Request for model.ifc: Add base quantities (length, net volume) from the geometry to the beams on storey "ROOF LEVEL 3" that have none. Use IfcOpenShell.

First a look at what the model holds.

```python
import ifcopenshell
import ifcopenshell.util.element
import ifcopenshell.util.unit

model = ifcopenshell.open("model.ifc")
print(model.schema)
for unit_type in ("LENGTHUNIT", "AREAUNIT", "VOLUMEUNIT"):
    print(unit_type, ifcopenshell.util.unit.calculate_unit_scale(model, unit_type))
storey = next(s for s in model.by_type("IfcBuildingStorey") if s.Name == "ROOF LEVEL 3")
beams = [e for e in ifcopenshell.util.element.get_decomposition(storey) if e.is_a("IfcBeam")]
for e in sorted(beams, key=lambda e: e.id()):
    print(e.id(), e.is_a(), e.Name, list(ifcopenshell.util.element.get_psets(e, qtos_only=True)), sep=" | ")
```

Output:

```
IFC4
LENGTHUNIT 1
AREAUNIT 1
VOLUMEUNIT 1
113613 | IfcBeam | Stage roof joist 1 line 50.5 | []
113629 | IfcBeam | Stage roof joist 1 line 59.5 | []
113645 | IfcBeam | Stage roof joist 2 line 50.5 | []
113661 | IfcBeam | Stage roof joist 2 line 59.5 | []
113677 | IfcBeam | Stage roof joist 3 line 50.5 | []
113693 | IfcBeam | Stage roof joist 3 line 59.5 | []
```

```python
import ifcopenshell
import ifcopenshell.api.pset
import ifcopenshell.geom
import ifcopenshell.util.element
import ifcopenshell.util.shape
import ifcopenshell.util.unit

model = ifcopenshell.open("model.ifc")
unit_scale = ifcopenshell.util.unit.calculate_unit_scale(model)
volume_scale = ifcopenshell.util.unit.calculate_unit_scale(model, "VOLUMEUNIT")
settings = ifcopenshell.geom.settings()

storey = next(s for s in model.by_type("IfcBuildingStorey") if s.Name == "ROOF LEVEL 3")
beams = [e for e in ifcopenshell.util.element.get_decomposition(storey) if e.is_a("IfcBeam")]

for e in sorted(beams, key=lambda e: e.id()):
    if ifcopenshell.util.element.get_psets(e, qtos_only=True, should_inherit=False):
        continue
    # Geometry comes back in metres, in the element's own axes.
    shape = ifcopenshell.geom.create_shape(settings, e)
    values = {
        "Length": ifcopenshell.util.shape.get_max_xyz(shape.geometry) / unit_scale,
        "NetVolume": ifcopenshell.util.shape.get_volume(shape.geometry) / volume_scale,
    }
    qto = ifcopenshell.api.pset.add_qto(model, product=e, name="Qto_BeamBaseQuantities")
    ifcopenshell.api.pset.edit_qto(model, qto=qto, properties=values)
    print(e.id(), {k: round(v, 3) for k, v in values.items()})

model.write("model_v2.ifc")
```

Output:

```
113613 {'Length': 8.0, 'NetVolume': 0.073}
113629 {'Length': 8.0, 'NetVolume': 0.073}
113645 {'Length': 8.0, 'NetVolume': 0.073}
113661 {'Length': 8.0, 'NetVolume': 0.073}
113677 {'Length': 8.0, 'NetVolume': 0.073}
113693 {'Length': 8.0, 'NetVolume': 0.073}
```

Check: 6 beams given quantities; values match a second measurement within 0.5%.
